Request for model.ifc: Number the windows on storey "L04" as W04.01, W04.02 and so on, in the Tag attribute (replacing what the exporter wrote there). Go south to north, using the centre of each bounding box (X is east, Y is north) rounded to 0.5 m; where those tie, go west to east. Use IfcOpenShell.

First a look at what the model holds.

```python
import ifcopenshell
import ifcopenshell.util.element
import ifcopenshell.util.placement

model = ifcopenshell.open("model.ifc")
print(model.schema)
storey = next(s for s in model.by_type("IfcBuildingStorey") if s.Name == "L04")
windows = [e for e in ifcopenshell.util.element.get_decomposition(storey) if e.is_a("IfcWindow")]
for e in sorted(windows, key=lambda e: e.id()):
    origin = ifcopenshell.util.placement.get_local_placement(e.ObjectPlacement)[:3, 3]
    print(e.id(), e.Tag, e.Name, origin.round(2) + 0.0, sep=" | ")
```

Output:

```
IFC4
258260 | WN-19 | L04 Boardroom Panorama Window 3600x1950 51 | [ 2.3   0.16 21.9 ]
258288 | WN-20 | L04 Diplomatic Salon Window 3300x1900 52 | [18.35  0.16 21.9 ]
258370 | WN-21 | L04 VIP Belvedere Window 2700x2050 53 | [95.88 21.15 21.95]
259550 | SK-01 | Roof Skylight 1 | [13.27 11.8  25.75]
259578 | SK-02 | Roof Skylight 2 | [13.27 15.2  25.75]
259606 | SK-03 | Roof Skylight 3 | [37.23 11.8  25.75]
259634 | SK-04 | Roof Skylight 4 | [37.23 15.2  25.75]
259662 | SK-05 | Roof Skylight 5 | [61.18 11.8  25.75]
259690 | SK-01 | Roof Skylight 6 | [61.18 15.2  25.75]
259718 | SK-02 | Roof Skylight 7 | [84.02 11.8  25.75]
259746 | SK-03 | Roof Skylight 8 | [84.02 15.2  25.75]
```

```python
import ifcopenshell
import ifcopenshell.geom
import ifcopenshell.util.element
import ifcopenshell.util.shape

model = ifcopenshell.open("model.ifc")
settings = ifcopenshell.geom.settings()
settings.set("use-world-coords", True)


def centre(element):
    shape = ifcopenshell.geom.create_shape(settings, element)
    return ifcopenshell.util.shape.get_bbox_centroid(shape.geometry)


storey = next(s for s in model.by_type("IfcBuildingStorey") if s.Name == "L04")
windows = [e for e in ifcopenshell.util.element.get_decomposition(storey) if e.is_a("IfcWindow")]

# Insertion points can sit at a corner or the storey origin, so sort by the geometry (in metres).
centres = {e: centre(e) for e in windows}
windows.sort(key=lambda e: (round(centres[e][1] / 0.5), centres[e][0]))

for i, e in enumerate(windows, start=1):
    number = f"W04.{i:02d}"
    e.Tag = number
    print(e.id(), number)

model.write("model_rev.ifc")
```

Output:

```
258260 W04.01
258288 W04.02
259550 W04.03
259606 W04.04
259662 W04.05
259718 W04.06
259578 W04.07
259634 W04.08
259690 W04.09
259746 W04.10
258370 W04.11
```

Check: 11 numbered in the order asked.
